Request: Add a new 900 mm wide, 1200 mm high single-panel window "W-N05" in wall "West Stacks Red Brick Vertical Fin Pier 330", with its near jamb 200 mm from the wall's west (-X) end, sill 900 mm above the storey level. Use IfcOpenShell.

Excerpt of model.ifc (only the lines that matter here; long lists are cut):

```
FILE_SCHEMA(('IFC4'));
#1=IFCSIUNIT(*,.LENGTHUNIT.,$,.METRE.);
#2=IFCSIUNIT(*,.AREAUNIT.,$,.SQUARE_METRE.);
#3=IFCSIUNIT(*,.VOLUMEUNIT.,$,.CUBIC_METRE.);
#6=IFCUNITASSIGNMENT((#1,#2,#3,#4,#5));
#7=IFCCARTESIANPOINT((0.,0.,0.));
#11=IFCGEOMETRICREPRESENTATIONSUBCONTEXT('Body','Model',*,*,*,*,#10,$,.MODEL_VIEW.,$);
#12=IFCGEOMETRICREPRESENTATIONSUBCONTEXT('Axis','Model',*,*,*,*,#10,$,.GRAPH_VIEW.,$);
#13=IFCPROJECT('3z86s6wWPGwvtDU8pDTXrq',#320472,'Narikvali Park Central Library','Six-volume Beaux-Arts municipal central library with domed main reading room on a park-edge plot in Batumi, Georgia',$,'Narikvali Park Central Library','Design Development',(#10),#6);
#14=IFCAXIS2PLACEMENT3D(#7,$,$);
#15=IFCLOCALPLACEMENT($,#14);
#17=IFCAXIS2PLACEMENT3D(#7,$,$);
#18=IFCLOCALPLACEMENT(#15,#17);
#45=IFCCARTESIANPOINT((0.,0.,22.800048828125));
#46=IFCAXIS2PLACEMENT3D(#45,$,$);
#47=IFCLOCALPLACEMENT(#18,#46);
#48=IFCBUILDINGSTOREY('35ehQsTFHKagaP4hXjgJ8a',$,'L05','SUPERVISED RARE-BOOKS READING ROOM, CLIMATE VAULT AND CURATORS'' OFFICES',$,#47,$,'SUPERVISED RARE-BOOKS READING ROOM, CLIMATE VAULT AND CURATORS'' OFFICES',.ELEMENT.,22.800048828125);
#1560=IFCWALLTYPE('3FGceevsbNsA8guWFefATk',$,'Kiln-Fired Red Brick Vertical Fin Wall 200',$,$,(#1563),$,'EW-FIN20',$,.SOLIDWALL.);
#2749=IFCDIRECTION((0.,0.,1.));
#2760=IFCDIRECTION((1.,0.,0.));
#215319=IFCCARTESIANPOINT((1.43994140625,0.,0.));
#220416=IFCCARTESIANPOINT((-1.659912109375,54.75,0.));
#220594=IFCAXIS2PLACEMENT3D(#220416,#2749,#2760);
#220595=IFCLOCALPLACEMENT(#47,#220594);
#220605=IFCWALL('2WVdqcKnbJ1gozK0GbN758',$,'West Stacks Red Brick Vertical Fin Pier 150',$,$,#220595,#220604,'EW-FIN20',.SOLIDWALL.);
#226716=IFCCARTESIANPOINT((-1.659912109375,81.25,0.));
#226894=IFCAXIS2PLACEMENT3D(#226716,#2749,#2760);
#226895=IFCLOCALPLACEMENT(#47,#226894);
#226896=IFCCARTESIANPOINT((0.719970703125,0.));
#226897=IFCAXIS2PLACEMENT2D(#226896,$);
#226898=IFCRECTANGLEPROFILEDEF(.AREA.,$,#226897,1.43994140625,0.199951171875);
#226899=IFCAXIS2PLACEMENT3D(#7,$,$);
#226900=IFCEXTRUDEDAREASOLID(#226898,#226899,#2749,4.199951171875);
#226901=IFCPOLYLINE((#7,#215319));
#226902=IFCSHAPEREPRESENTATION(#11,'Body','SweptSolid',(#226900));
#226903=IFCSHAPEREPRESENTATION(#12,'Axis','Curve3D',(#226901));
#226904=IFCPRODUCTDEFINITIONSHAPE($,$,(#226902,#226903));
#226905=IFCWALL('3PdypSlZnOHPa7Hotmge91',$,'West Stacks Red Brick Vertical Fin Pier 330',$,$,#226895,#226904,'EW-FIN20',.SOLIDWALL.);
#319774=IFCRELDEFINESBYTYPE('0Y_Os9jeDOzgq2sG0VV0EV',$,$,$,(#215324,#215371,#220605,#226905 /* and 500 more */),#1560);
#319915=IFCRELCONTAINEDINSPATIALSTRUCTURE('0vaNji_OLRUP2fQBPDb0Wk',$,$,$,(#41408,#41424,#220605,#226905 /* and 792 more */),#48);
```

```python
import numpy as np
import ifcopenshell
import ifcopenshell.api.feature
import ifcopenshell.api.geometry
import ifcopenshell.api.root
import ifcopenshell.api.spatial
import ifcopenshell.geom
import ifcopenshell.util.element
import ifcopenshell.util.placement
import ifcopenshell.util.representation
import ifcopenshell.util.shape
import ifcopenshell.util.unit

model = ifcopenshell.open("model.ifc")
unit_scale = ifcopenshell.util.unit.calculate_unit_scale(model)
settings = ifcopenshell.geom.settings()


def volume(element):
    """Net volume in cubic metres, openings subtracted."""
    shape = ifcopenshell.geom.create_shape(settings, element)
    return ifcopenshell.util.shape.get_volume(shape.geometry)


wall = model.by_guid("3PdypSlZnOHPa7Hotmge91")
storey = ifcopenshell.util.element.get_container(wall, ifc_class="IfcBuildingStorey")
context = ifcopenshell.util.representation.get_context(model, "Model", "Body", "MODEL_VIEW")
before = volume(wall)

width, height, from_end, sill = 0.9, 1.2, 0.2, 0.9  # metres

# The wall runs along its own X axis, and the end named is its -X end.
wall_shape = ifcopenshell.geom.create_shape(settings, wall)
x, y, z = ifcopenshell.util.shape.get_vertices(wall_shape.geometry).T
start = x.min() + from_end
face, thickness = float(y.min()), float(y.max() - y.min())
wall_matrix = ifcopenshell.util.placement.get_local_placement(wall.ObjectPlacement)
level = ifcopenshell.util.placement.get_local_placement(storey.ObjectPlacement)[2, 3]


def in_wall(x, y):
    """Placement at x, y metres in the wall's axes, at sill height."""
    matrix = wall_matrix.copy()
    matrix[:, 3] = wall_matrix @ np.array([x / unit_scale, y / unit_scale, 0.0, 1.0])
    matrix[2, 3] = level + sill / unit_scale
    return matrix


# Opening: a box that overshoots both wall faces by 50 mm.
opening = ifcopenshell.api.root.create_entity(model, ifc_class="IfcOpeningElement", predefined_type="OPENING")
box = ifcopenshell.api.geometry.add_wall_representation(
    model, context=context, length=width, height=height, thickness=thickness + 0.1
)
ifcopenshell.api.geometry.assign_representation(model, product=opening, representation=box)
ifcopenshell.api.geometry.edit_object_placement(model, product=opening, matrix=in_wall(start, face - 0.05), is_si=False)
ifcopenshell.api.feature.add_feature(model, feature=opening, element=wall)

window = ifcopenshell.api.root.create_entity(model, ifc_class="IfcWindow", name="W-N05", predefined_type="WINDOW")
window.OverallWidth, window.OverallHeight = width / unit_scale, height / unit_scale
window.PartitioningType = "SINGLE_PANEL"
body = ifcopenshell.api.geometry.add_window_representation(
    model,
    context=context,
    overall_width=window.OverallWidth,
    overall_height=window.OverallHeight,
    partition_type="SINGLE_PANEL",
)
ifcopenshell.api.geometry.assign_representation(model, product=window, representation=body)
ifcopenshell.api.spatial.assign_container(model, products=[window], relating_structure=storey)
ifcopenshell.api.feature.add_filling(model, opening=opening, element=window)

# Centre the window in the wall's thickness.
ifcopenshell.api.geometry.edit_object_placement(model, product=window, matrix=in_wall(start, face), is_si=False)
window_shape = ifcopenshell.geom.create_shape(settings, window)
depth = ifcopenshell.util.shape.get_vertices(window_shape.geometry)[:, 1]
offset = face + thickness / 2 - (depth.min() + depth.max()) / 2
ifcopenshell.api.geometry.edit_object_placement(model, product=window, matrix=in_wall(start, offset), is_si=False)

after = volume(wall)

print(f"wall volume {before:.3f} -> {after:.3f} m3")

model.write("model-out.ifc")
```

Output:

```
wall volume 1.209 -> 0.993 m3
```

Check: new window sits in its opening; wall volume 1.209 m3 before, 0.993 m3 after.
